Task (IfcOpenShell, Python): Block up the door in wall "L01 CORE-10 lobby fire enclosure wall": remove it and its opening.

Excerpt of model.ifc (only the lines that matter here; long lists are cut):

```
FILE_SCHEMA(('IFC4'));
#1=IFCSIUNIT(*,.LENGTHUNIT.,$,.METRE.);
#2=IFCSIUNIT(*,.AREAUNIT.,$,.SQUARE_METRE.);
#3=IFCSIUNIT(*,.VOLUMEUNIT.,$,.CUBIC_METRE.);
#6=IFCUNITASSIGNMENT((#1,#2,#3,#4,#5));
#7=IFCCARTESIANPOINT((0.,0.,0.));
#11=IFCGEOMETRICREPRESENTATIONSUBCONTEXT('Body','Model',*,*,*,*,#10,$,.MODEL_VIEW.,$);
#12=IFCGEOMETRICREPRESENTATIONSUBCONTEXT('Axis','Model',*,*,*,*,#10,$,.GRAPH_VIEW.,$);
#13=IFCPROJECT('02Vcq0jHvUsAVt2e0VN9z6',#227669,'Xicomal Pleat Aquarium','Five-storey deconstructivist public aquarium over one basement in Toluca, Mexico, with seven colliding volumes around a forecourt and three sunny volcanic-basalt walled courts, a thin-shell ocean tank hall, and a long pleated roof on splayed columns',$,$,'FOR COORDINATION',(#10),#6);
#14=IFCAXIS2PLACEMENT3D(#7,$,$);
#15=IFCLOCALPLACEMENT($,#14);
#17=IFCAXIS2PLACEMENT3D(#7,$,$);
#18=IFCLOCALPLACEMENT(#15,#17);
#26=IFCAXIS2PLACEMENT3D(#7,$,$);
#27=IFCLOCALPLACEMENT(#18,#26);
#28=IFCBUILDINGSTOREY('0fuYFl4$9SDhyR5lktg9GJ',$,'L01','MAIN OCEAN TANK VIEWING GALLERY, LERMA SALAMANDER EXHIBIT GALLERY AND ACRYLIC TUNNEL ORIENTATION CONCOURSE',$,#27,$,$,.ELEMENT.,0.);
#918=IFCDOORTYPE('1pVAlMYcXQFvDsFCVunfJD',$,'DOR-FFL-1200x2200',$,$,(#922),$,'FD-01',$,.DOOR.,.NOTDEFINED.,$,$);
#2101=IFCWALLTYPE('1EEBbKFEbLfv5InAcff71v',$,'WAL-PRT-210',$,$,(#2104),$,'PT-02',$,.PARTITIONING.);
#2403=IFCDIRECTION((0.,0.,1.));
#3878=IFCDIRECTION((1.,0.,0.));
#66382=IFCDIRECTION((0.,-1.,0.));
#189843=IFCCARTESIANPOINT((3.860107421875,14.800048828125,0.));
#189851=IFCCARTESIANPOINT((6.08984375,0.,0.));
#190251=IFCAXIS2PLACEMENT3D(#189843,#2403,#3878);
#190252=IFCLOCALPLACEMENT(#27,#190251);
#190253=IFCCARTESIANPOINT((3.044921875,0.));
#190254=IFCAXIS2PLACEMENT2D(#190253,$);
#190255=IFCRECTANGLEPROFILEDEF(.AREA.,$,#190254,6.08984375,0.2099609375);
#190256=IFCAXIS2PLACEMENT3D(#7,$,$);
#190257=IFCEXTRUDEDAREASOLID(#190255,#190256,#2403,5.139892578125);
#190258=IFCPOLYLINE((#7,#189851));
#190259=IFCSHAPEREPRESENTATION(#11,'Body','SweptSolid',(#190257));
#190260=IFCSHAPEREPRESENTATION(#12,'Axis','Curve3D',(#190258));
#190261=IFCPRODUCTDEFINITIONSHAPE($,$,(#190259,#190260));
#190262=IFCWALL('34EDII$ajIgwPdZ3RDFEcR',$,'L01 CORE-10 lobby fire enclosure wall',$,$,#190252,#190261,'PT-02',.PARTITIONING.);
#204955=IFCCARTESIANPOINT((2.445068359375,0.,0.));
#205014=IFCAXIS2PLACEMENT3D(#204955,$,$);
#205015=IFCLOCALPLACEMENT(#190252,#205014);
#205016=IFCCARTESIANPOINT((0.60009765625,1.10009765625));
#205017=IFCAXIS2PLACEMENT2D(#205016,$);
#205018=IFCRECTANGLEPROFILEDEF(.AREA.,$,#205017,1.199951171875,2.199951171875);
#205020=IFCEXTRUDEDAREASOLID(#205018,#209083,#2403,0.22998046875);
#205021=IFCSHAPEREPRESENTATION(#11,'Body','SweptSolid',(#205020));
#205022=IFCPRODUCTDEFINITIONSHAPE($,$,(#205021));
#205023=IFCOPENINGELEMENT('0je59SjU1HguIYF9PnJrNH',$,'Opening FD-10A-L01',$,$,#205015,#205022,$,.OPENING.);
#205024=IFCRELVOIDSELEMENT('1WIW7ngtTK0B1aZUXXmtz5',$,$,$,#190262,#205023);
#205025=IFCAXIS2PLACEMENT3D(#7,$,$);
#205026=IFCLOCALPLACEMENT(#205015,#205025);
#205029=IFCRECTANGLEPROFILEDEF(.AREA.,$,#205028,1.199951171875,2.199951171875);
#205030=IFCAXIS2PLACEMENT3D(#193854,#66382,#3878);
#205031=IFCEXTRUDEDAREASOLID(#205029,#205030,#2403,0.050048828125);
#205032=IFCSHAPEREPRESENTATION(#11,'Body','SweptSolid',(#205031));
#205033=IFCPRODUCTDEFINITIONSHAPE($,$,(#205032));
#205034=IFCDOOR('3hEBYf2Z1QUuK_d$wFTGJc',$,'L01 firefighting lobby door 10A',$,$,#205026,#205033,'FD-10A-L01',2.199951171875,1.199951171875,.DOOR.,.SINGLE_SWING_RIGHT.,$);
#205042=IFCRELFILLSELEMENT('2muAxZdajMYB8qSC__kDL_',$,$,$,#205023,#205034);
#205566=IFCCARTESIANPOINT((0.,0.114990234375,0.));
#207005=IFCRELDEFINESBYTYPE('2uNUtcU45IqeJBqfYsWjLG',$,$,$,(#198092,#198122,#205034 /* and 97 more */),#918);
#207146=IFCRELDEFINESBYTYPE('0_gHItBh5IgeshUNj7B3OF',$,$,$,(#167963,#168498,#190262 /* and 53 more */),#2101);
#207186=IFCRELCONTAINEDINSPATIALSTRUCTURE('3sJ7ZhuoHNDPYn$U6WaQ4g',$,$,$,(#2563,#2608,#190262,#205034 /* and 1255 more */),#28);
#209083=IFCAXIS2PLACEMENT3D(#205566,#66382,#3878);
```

```python
import ifcopenshell
import ifcopenshell.api.feature
import ifcopenshell.api.root
import ifcopenshell.geom
import ifcopenshell.util.shape

model = ifcopenshell.open("model.ifc")
settings = ifcopenshell.geom.settings()


def volume(element):
    """Net volume in cubic metres, openings subtracted."""
    shape = ifcopenshell.geom.create_shape(settings, element)
    return ifcopenshell.util.shape.get_volume(shape.geometry)


door = model.by_guid("3hEBYf2Z1QUuK_d$wFTGJc")
opening = door.FillsVoids[0].RelatingOpeningElement
wall = opening.VoidsElements[0].RelatingBuildingElement
before = volume(wall)

ifcopenshell.api.root.remove_product(model, product=door)
ifcopenshell.api.feature.remove_feature(model, feature=opening)

after = volume(wall)

print(f"wall volume {before:.3f} -> {after:.3f} m3")

model.write("model_updated.ifc")
```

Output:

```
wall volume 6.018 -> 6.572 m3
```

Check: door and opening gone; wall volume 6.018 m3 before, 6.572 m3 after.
